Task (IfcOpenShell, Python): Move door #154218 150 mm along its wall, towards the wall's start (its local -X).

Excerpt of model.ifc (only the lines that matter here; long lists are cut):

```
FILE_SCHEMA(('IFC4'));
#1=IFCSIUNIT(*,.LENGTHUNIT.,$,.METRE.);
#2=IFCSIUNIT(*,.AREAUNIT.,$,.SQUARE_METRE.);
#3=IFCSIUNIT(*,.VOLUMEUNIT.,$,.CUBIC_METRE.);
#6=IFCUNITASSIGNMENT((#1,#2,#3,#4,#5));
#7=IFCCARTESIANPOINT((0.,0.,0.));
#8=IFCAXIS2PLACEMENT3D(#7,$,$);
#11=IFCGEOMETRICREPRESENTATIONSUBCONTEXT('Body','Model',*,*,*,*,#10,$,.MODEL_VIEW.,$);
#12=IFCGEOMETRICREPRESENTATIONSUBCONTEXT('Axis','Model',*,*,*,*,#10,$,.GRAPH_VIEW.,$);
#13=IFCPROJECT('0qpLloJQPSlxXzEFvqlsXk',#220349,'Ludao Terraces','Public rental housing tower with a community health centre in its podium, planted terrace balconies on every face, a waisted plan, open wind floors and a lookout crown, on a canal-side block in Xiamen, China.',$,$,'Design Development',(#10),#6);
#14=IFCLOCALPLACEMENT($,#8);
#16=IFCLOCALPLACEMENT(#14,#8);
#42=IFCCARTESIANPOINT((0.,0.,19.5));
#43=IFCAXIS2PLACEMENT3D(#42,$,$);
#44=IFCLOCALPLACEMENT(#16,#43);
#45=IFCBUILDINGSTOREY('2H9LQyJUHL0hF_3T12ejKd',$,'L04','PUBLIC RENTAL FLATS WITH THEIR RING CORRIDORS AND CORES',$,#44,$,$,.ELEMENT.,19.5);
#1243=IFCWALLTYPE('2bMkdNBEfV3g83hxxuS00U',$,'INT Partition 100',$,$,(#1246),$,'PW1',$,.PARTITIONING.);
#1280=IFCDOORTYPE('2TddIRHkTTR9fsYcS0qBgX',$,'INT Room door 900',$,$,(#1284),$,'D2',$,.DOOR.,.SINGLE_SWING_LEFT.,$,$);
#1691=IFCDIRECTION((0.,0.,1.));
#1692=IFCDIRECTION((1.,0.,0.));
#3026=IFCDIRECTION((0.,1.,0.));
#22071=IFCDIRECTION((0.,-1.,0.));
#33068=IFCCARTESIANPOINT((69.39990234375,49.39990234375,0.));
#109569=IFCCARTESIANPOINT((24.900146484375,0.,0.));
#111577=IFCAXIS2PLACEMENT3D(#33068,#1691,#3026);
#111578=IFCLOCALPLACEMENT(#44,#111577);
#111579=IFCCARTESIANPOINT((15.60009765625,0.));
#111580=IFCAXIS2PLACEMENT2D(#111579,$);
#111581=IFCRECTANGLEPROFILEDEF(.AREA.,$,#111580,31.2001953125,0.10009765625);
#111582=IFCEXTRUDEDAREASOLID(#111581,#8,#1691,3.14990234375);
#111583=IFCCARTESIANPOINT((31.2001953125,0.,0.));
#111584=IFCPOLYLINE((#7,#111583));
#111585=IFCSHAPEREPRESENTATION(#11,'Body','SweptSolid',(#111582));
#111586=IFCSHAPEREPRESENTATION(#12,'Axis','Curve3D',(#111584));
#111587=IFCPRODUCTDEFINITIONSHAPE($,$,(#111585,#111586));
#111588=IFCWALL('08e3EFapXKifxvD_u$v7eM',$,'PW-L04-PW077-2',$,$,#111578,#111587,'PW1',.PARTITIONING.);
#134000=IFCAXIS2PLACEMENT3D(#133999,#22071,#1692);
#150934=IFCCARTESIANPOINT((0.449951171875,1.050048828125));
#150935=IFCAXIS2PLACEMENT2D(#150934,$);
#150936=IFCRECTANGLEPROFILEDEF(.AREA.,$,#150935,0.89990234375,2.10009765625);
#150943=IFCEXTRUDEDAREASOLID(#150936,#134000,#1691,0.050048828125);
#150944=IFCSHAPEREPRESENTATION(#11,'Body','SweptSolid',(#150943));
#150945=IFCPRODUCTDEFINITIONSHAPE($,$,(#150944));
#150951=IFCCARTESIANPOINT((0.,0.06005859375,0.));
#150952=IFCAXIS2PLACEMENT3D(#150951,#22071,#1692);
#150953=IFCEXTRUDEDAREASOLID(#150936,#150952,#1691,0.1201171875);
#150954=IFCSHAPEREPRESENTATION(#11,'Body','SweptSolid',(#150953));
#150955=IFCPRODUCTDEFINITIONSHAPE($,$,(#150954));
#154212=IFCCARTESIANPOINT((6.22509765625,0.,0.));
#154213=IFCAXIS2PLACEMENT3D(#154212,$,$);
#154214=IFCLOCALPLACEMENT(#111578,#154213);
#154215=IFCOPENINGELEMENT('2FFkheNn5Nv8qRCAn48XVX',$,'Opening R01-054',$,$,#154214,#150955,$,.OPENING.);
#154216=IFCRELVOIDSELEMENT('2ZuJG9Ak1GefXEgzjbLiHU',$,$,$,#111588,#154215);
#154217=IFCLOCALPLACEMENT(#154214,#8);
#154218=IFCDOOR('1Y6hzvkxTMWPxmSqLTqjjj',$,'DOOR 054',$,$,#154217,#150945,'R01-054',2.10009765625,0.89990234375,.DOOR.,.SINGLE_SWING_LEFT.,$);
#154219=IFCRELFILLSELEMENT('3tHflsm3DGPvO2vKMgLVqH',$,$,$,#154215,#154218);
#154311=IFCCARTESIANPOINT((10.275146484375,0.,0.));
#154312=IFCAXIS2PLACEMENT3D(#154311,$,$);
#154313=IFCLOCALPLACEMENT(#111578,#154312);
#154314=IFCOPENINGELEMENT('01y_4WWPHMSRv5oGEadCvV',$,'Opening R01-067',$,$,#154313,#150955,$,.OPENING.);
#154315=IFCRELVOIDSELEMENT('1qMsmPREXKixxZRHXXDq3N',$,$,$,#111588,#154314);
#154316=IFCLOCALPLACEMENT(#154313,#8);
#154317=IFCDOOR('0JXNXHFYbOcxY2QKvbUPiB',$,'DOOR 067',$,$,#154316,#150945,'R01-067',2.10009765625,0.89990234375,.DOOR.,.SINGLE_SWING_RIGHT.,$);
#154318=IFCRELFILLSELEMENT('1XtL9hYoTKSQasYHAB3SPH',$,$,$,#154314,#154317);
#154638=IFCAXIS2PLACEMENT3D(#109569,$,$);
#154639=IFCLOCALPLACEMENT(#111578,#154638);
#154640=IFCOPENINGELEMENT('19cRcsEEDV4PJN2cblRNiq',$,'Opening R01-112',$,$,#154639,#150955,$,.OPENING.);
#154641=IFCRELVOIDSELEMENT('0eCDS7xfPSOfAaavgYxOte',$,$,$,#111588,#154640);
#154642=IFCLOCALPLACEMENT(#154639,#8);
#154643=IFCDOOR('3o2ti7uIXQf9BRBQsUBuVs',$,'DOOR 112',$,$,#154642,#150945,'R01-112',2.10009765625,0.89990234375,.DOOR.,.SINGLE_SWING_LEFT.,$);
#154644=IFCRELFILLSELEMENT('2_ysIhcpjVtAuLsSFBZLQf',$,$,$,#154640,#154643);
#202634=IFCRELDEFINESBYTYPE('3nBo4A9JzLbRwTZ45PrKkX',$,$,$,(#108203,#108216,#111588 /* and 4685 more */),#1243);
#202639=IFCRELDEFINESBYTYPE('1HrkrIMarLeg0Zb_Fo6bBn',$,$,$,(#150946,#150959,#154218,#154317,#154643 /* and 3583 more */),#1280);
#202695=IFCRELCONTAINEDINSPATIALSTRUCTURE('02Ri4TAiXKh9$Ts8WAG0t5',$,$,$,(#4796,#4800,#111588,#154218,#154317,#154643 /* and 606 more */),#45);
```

```python
import ifcopenshell
import ifcopenshell.api.geometry
import ifcopenshell.util.placement

model = ifcopenshell.open("model.ifc")

door = model.by_id(154218)
opening = door.FillsVoids[0].RelatingOpeningElement
wall = opening.VoidsElements[0].RelatingBuildingElement

wall_matrix = ifcopenshell.util.placement.get_local_placement(wall.ObjectPlacement)
shift = wall_matrix[:3, 0] * -0.15
before = ifcopenshell.util.placement.get_local_placement(door.ObjectPlacement)[:3, 3].copy()

# The door is placed relative to its opening, so it follows when the opening moves.
matrix = ifcopenshell.util.placement.get_local_placement(opening.ObjectPlacement)
matrix[:3, 3] += shift
ifcopenshell.api.geometry.edit_object_placement(
    model, product=opening, matrix=matrix, is_si=False, should_transform_children=True
)

after = ifcopenshell.util.placement.get_local_placement(door.ObjectPlacement)[:3, 3]
print("door moved by", (after - before).round(3) + 0.0)

model.write("model_rev.ifc")
```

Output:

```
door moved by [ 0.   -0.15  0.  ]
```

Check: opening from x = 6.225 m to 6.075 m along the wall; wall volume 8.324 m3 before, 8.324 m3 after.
